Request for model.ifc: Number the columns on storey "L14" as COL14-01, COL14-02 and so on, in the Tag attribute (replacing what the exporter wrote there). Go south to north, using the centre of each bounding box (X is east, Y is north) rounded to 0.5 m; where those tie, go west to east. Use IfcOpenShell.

First a look at what the model holds.

```python
import ifcopenshell
import ifcopenshell.util.element
import ifcopenshell.util.placement

model = ifcopenshell.open("model.ifc")
print(model.schema)
storey = next(s for s in model.by_type("IfcBuildingStorey") if s.Name == "L14")
columns = [e for e in ifcopenshell.util.element.get_decomposition(storey) if e.is_a("IfcColumn")]
for e in sorted(columns, key=lambda e: e.id()):
    origin = ifcopenshell.util.placement.get_local_placement(e.ObjectPlacement)[:3, 3]
    print(e.id(), e.Tag, e.Name, origin.round(2) + 0.0, sep=" | ")
```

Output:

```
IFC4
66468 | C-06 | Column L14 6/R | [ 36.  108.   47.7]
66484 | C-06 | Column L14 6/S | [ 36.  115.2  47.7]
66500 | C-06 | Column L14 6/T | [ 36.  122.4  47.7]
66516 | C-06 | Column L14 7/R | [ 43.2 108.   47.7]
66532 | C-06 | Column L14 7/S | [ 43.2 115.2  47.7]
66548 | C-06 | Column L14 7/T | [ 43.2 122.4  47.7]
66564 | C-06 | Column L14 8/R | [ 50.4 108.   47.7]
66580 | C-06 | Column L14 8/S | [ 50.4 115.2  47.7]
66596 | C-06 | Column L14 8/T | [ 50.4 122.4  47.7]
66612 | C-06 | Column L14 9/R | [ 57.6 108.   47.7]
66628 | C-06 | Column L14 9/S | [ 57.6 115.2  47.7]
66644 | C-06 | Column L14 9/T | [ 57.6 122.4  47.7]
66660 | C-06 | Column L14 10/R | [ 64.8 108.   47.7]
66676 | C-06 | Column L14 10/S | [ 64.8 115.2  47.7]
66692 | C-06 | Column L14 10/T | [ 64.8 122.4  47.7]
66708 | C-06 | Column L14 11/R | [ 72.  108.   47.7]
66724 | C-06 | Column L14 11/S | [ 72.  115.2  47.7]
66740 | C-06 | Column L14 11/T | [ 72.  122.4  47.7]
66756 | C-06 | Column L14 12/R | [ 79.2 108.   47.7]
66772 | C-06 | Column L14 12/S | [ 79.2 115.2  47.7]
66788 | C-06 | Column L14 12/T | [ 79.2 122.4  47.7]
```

```python
import ifcopenshell
import ifcopenshell.geom
import ifcopenshell.util.element
import ifcopenshell.util.shape

model = ifcopenshell.open("model.ifc")
settings = ifcopenshell.geom.settings()
settings.set("use-world-coords", True)


def centre(element):
    shape = ifcopenshell.geom.create_shape(settings, element)
    return ifcopenshell.util.shape.get_bbox_centroid(shape.geometry)


storey = next(s for s in model.by_type("IfcBuildingStorey") if s.Name == "L14")
columns = [e for e in ifcopenshell.util.element.get_decomposition(storey) if e.is_a("IfcColumn")]

# Insertion points can sit at a corner or the storey origin, so sort by the geometry (in metres).
centres = {e: centre(e) for e in columns}
columns.sort(key=lambda e: (round(centres[e][1] / 0.5), centres[e][0]))

for i, e in enumerate(columns, start=1):
    number = f"COL14-{i:02d}"
    e.Tag = number
    print(e.id(), number)

model.write("model_updated.ifc")
```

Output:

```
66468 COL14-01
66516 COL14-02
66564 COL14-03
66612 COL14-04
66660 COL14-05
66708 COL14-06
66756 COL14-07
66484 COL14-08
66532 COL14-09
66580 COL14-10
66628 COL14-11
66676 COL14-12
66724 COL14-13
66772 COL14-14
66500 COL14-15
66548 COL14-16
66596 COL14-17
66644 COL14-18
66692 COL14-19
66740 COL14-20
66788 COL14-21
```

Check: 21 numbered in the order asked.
